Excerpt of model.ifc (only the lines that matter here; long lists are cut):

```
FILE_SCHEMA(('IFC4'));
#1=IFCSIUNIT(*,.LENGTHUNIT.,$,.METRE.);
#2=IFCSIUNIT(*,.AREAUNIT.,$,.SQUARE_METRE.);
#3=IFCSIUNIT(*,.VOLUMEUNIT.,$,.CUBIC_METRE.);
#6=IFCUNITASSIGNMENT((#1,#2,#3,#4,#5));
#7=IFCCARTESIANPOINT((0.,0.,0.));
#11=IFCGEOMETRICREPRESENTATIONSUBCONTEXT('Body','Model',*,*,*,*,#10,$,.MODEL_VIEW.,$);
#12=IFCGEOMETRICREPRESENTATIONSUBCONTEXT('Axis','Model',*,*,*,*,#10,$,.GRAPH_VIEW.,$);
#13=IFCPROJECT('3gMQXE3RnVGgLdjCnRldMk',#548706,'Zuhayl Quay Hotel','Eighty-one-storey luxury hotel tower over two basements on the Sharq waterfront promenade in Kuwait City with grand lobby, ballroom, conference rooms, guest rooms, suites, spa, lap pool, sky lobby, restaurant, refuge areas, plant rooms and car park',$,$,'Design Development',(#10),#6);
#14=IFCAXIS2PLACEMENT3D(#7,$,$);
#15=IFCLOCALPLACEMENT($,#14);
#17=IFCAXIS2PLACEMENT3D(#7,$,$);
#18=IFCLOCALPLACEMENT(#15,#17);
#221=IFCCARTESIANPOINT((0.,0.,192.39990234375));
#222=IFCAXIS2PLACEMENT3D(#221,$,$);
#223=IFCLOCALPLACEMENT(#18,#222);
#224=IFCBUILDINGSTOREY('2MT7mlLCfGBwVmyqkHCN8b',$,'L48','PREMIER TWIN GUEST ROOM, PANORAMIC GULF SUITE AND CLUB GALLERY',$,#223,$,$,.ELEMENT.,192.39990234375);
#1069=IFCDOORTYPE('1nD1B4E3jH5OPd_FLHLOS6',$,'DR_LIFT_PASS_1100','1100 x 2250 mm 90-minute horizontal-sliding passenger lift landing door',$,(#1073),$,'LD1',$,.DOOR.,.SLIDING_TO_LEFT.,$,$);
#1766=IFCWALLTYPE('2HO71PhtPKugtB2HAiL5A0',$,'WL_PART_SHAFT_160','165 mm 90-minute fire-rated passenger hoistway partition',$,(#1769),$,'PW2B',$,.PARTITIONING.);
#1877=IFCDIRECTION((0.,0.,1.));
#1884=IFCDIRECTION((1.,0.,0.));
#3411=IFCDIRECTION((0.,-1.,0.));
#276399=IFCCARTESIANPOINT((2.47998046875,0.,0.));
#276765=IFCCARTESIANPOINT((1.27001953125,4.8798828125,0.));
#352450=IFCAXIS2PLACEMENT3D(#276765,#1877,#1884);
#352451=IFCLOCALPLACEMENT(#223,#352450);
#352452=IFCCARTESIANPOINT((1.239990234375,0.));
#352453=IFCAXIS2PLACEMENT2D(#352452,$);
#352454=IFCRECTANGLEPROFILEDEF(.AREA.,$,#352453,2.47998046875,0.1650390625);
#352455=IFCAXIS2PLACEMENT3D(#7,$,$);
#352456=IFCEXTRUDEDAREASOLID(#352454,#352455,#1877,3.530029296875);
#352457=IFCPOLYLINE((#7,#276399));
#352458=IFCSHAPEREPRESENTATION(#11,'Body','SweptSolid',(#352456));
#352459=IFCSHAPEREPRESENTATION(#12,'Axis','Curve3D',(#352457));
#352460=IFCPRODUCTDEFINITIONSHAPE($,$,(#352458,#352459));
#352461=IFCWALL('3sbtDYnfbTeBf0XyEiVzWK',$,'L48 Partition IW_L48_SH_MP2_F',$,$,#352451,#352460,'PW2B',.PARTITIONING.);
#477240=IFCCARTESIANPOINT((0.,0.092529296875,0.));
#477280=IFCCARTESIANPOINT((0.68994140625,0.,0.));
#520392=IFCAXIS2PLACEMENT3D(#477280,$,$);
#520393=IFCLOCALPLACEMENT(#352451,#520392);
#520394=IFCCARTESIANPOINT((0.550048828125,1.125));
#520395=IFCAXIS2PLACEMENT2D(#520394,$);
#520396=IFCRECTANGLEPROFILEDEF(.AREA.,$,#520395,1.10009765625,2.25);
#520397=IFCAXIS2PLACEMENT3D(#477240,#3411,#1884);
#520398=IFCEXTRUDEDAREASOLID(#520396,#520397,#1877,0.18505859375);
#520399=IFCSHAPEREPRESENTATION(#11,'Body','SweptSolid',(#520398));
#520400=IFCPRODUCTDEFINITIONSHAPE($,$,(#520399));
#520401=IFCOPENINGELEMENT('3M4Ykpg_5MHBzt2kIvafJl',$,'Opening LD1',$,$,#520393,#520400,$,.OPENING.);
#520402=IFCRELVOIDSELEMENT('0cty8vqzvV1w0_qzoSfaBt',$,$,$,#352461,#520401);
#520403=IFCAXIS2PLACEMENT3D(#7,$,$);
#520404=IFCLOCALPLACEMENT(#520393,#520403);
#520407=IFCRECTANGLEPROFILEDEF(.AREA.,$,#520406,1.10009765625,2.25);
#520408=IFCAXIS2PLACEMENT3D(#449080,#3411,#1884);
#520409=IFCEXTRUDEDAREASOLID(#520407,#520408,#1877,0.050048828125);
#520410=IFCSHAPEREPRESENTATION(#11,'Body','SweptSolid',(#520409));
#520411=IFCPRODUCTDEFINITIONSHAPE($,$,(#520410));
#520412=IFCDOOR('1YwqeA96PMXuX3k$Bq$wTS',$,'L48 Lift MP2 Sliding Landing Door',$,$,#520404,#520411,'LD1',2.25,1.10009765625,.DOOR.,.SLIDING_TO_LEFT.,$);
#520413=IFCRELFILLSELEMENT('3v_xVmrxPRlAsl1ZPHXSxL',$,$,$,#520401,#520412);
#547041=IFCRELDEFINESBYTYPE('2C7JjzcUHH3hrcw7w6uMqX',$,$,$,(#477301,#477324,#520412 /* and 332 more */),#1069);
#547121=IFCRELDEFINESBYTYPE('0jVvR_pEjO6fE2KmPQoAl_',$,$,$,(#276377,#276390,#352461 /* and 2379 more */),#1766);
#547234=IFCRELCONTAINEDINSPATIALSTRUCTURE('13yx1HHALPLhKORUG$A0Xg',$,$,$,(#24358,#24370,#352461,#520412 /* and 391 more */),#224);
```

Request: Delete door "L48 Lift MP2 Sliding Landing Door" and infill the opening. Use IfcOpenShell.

```python
import ifcopenshell
import ifcopenshell.api.feature
import ifcopenshell.api.root
import ifcopenshell.geom
import ifcopenshell.util.shape

model = ifcopenshell.open("model.ifc")
settings = ifcopenshell.geom.settings()


def volume(element):
    """Net volume in cubic metres, openings subtracted."""
    shape = ifcopenshell.geom.create_shape(settings, element)
    return ifcopenshell.util.shape.get_volume(shape.geometry)


door = model.by_guid("1YwqeA96PMXuX3k$Bq$wTS")
opening = door.FillsVoids[0].RelatingOpeningElement
wall = opening.VoidsElements[0].RelatingBuildingElement
before = volume(wall)

ifcopenshell.api.root.remove_product(model, product=door)
ifcopenshell.api.feature.remove_feature(model, feature=opening)

after = volume(wall)

print(f"wall volume {before:.3f} -> {after:.3f} m3")

model.write("model_updated.ifc")
```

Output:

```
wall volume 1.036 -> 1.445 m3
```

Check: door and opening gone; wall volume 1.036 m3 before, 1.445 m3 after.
